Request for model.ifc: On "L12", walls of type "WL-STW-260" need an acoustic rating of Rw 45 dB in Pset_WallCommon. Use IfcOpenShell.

First a look at what the model holds.

```python
import ifcopenshell
import ifcopenshell.util.element

model = ifcopenshell.open("model.ifc")
print(model.schema)
storey = next(s for s in model.by_type("IfcBuildingStorey") if s.Name == "L12")
walls = [e for e in ifcopenshell.util.element.get_decomposition(storey) if e.is_a("IfcWall")]
seen = {}
for e in walls:
    element_type = ifcopenshell.util.element.get_type(e)
    key = (element_type.Name if element_type != e and element_type else None, ifcopenshell.util.element.get_pset(e, "Pset_WallCommon", "AcousticRating"))
    seen[key] = seen.get(key, 0) + 1
for (name, value), count in sorted(seen.items(), key=str):
    print(count, "x", name, "|", value)
```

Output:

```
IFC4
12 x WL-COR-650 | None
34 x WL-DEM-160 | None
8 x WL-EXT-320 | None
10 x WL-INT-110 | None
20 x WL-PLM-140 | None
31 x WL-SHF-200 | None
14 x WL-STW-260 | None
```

```python
import ifcopenshell
import ifcopenshell.api.pset
import ifcopenshell.util.element

model = ifcopenshell.open("model.ifc")

storey = next(s for s in model.by_type("IfcBuildingStorey") if s.Name == "L12")
walls = [e for e in ifcopenshell.util.element.get_decomposition(storey) if e.is_a("IfcWall")]

count = 0
for e in walls:
    element_type = ifcopenshell.util.element.get_type(e)
    if element_type in (None, e) or element_type.Name != "WL-STW-260":
        continue
    found = ifcopenshell.util.element.get_pset(e, "Pset_WallCommon", should_inherit=False)
    if found:
        pset = model.by_id(found["id"])
        if len(ifcopenshell.util.element.get_elements_by_pset(pset)) > 1:
            pset = ifcopenshell.api.pset.unshare_pset(model, products=[e], pset=pset)[0]
    else:
        pset = ifcopenshell.api.pset.add_pset(model, product=e, name="Pset_WallCommon")
    ifcopenshell.api.pset.edit_pset(model, pset=pset, properties={"AcousticRating": "Rw 45 dB"})
    count += 1

print(count, "walls updated")

model.write("model_rev.ifc")
```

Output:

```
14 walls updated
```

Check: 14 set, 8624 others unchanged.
